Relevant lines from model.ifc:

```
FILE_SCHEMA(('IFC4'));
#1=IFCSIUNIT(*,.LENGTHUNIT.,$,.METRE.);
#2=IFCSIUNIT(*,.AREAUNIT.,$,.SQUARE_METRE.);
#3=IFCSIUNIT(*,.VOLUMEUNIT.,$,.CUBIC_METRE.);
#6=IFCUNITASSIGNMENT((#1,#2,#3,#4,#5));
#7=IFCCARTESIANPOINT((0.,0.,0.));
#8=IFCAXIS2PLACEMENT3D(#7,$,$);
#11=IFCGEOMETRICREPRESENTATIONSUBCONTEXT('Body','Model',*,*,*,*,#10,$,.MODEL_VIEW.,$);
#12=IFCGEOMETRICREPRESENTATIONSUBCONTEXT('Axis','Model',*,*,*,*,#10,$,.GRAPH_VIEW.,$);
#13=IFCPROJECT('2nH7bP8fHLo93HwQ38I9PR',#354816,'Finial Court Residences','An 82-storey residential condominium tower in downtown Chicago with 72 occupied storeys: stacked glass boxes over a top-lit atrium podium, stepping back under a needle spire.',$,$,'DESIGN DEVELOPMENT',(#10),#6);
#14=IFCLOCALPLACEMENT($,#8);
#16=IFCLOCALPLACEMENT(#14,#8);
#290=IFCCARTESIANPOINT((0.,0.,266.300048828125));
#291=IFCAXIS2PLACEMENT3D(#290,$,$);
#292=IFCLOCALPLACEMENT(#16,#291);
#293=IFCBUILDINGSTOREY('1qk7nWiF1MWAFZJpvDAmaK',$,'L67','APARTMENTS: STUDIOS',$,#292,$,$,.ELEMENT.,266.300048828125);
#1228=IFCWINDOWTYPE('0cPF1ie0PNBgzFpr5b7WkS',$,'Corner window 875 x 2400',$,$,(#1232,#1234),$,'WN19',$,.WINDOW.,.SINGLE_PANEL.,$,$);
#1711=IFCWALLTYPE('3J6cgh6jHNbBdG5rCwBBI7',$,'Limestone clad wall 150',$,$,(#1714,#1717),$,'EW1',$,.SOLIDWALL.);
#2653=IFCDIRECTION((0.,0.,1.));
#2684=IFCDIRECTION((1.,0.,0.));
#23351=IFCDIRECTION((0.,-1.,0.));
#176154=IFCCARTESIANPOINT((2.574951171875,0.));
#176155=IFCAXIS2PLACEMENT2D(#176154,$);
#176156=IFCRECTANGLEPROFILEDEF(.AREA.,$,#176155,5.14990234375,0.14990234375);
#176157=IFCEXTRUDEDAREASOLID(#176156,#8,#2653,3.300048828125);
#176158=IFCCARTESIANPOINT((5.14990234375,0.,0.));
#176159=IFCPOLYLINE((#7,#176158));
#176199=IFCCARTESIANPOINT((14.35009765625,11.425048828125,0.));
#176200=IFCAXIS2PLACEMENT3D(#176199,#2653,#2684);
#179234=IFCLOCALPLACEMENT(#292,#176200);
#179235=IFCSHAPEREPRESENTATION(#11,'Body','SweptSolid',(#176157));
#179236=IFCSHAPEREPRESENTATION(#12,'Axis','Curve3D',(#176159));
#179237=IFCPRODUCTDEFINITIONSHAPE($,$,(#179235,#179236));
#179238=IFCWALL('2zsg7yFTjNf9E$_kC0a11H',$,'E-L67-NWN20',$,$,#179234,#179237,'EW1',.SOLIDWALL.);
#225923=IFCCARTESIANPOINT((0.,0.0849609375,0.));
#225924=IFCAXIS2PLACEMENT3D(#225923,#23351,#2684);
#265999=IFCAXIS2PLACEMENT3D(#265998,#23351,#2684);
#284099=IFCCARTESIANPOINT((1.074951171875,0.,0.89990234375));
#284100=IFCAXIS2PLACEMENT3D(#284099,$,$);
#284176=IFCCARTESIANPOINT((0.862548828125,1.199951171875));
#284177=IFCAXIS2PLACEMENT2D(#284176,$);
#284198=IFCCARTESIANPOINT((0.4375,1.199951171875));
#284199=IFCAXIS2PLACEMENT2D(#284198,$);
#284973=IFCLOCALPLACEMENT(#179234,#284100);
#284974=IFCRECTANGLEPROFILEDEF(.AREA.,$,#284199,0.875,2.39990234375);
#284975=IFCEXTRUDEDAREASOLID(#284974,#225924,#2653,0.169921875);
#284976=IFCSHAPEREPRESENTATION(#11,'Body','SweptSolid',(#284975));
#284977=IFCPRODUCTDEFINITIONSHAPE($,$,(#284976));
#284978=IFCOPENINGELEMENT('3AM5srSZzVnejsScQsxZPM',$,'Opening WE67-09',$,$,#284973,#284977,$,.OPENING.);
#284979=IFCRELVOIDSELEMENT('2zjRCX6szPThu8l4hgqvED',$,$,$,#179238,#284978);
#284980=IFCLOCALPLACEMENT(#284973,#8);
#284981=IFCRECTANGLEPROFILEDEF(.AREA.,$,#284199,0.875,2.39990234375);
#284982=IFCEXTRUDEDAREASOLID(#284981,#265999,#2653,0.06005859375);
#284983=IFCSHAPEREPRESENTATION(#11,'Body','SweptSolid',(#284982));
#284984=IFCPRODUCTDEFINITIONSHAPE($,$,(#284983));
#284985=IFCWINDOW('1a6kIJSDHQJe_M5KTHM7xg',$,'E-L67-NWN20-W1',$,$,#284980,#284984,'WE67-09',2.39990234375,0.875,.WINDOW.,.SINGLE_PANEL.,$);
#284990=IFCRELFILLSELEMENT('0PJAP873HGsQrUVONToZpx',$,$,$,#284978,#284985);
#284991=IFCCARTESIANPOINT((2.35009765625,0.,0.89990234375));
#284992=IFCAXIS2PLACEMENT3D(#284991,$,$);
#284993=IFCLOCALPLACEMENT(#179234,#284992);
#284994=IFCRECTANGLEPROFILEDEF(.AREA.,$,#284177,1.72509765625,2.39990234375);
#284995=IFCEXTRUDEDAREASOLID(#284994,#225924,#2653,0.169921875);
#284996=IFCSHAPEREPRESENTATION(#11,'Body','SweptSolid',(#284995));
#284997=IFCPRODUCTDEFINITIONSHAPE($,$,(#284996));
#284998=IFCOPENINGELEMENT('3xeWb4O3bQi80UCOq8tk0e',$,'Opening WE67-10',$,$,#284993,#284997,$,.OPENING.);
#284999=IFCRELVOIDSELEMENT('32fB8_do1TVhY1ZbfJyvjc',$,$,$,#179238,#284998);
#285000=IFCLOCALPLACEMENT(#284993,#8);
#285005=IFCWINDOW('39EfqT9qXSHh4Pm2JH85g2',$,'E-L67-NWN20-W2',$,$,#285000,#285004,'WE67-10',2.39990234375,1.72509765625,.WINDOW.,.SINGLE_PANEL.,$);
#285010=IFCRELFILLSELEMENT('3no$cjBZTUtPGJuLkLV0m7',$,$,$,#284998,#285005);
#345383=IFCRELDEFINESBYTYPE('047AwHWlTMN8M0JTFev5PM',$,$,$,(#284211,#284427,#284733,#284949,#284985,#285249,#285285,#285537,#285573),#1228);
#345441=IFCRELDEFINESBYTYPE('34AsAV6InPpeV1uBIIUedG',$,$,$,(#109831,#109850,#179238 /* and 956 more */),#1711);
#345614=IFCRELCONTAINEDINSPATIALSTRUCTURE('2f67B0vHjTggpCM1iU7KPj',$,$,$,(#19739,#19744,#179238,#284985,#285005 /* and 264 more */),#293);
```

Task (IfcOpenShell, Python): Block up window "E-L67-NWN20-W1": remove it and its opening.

```python
import ifcopenshell
import ifcopenshell.api.feature
import ifcopenshell.api.root
import ifcopenshell.geom
import ifcopenshell.util.shape

model = ifcopenshell.open("model.ifc")
settings = ifcopenshell.geom.settings()


def volume(element):
    """Net volume in cubic metres, openings subtracted."""
    shape = ifcopenshell.geom.create_shape(settings, element)
    return ifcopenshell.util.shape.get_volume(shape.geometry)


window = model.by_guid("1a6kIJSDHQJe_M5KTHM7xg")
opening = window.FillsVoids[0].RelatingOpeningElement
wall = opening.VoidsElements[0].RelatingBuildingElement
before = volume(wall)

ifcopenshell.api.root.remove_product(model, product=window)
ifcopenshell.api.feature.remove_feature(model, feature=opening)

after = volume(wall)

print(f"wall volume {before:.3f} -> {after:.3f} m3")

model.write("model-out.ifc")
```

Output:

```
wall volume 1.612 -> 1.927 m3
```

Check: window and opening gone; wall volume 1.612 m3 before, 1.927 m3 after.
